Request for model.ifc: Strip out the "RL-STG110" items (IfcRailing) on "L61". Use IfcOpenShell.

First a look at what the model holds.

```python
import ifcopenshell
import ifcopenshell.util.element

model = ifcopenshell.open("model.ifc")
print(model.schema)
storey = next(s for s in model.by_type("IfcBuildingStorey") if s.Name == "L61")
railings = [e for e in ifcopenshell.util.element.get_decomposition(storey) if e.is_a("IfcRailing")]
seen = {}
for e in railings:
    element_type = ifcopenshell.util.element.get_type(e)
    name = element_type.Name if element_type not in (None, e) else None
    seen[name] = seen.get(name, 0) + 1
for name, count in sorted(seen.items(), key=str):
    print(count, "x", name)
```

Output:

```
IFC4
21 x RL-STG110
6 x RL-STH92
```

```python
import ifcopenshell
import ifcopenshell.api.root
import ifcopenshell.util.element

model = ifcopenshell.open("model.ifc")

storey = next(s for s in model.by_type("IfcBuildingStorey") if s.Name == "L61")
railings = [e for e in ifcopenshell.util.element.get_decomposition(storey) if e.is_a("IfcRailing")]
targets = [e for e in railings if (t := ifcopenshell.util.element.get_type(e)) not in (None, e) and t.Name == "RL-STG110"]

for e in targets:
    ifcopenshell.api.root.remove_product(model, product=e)
print(len(targets), "removed")

model.write("model_updated.ifc")
```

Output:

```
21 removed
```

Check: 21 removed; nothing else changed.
